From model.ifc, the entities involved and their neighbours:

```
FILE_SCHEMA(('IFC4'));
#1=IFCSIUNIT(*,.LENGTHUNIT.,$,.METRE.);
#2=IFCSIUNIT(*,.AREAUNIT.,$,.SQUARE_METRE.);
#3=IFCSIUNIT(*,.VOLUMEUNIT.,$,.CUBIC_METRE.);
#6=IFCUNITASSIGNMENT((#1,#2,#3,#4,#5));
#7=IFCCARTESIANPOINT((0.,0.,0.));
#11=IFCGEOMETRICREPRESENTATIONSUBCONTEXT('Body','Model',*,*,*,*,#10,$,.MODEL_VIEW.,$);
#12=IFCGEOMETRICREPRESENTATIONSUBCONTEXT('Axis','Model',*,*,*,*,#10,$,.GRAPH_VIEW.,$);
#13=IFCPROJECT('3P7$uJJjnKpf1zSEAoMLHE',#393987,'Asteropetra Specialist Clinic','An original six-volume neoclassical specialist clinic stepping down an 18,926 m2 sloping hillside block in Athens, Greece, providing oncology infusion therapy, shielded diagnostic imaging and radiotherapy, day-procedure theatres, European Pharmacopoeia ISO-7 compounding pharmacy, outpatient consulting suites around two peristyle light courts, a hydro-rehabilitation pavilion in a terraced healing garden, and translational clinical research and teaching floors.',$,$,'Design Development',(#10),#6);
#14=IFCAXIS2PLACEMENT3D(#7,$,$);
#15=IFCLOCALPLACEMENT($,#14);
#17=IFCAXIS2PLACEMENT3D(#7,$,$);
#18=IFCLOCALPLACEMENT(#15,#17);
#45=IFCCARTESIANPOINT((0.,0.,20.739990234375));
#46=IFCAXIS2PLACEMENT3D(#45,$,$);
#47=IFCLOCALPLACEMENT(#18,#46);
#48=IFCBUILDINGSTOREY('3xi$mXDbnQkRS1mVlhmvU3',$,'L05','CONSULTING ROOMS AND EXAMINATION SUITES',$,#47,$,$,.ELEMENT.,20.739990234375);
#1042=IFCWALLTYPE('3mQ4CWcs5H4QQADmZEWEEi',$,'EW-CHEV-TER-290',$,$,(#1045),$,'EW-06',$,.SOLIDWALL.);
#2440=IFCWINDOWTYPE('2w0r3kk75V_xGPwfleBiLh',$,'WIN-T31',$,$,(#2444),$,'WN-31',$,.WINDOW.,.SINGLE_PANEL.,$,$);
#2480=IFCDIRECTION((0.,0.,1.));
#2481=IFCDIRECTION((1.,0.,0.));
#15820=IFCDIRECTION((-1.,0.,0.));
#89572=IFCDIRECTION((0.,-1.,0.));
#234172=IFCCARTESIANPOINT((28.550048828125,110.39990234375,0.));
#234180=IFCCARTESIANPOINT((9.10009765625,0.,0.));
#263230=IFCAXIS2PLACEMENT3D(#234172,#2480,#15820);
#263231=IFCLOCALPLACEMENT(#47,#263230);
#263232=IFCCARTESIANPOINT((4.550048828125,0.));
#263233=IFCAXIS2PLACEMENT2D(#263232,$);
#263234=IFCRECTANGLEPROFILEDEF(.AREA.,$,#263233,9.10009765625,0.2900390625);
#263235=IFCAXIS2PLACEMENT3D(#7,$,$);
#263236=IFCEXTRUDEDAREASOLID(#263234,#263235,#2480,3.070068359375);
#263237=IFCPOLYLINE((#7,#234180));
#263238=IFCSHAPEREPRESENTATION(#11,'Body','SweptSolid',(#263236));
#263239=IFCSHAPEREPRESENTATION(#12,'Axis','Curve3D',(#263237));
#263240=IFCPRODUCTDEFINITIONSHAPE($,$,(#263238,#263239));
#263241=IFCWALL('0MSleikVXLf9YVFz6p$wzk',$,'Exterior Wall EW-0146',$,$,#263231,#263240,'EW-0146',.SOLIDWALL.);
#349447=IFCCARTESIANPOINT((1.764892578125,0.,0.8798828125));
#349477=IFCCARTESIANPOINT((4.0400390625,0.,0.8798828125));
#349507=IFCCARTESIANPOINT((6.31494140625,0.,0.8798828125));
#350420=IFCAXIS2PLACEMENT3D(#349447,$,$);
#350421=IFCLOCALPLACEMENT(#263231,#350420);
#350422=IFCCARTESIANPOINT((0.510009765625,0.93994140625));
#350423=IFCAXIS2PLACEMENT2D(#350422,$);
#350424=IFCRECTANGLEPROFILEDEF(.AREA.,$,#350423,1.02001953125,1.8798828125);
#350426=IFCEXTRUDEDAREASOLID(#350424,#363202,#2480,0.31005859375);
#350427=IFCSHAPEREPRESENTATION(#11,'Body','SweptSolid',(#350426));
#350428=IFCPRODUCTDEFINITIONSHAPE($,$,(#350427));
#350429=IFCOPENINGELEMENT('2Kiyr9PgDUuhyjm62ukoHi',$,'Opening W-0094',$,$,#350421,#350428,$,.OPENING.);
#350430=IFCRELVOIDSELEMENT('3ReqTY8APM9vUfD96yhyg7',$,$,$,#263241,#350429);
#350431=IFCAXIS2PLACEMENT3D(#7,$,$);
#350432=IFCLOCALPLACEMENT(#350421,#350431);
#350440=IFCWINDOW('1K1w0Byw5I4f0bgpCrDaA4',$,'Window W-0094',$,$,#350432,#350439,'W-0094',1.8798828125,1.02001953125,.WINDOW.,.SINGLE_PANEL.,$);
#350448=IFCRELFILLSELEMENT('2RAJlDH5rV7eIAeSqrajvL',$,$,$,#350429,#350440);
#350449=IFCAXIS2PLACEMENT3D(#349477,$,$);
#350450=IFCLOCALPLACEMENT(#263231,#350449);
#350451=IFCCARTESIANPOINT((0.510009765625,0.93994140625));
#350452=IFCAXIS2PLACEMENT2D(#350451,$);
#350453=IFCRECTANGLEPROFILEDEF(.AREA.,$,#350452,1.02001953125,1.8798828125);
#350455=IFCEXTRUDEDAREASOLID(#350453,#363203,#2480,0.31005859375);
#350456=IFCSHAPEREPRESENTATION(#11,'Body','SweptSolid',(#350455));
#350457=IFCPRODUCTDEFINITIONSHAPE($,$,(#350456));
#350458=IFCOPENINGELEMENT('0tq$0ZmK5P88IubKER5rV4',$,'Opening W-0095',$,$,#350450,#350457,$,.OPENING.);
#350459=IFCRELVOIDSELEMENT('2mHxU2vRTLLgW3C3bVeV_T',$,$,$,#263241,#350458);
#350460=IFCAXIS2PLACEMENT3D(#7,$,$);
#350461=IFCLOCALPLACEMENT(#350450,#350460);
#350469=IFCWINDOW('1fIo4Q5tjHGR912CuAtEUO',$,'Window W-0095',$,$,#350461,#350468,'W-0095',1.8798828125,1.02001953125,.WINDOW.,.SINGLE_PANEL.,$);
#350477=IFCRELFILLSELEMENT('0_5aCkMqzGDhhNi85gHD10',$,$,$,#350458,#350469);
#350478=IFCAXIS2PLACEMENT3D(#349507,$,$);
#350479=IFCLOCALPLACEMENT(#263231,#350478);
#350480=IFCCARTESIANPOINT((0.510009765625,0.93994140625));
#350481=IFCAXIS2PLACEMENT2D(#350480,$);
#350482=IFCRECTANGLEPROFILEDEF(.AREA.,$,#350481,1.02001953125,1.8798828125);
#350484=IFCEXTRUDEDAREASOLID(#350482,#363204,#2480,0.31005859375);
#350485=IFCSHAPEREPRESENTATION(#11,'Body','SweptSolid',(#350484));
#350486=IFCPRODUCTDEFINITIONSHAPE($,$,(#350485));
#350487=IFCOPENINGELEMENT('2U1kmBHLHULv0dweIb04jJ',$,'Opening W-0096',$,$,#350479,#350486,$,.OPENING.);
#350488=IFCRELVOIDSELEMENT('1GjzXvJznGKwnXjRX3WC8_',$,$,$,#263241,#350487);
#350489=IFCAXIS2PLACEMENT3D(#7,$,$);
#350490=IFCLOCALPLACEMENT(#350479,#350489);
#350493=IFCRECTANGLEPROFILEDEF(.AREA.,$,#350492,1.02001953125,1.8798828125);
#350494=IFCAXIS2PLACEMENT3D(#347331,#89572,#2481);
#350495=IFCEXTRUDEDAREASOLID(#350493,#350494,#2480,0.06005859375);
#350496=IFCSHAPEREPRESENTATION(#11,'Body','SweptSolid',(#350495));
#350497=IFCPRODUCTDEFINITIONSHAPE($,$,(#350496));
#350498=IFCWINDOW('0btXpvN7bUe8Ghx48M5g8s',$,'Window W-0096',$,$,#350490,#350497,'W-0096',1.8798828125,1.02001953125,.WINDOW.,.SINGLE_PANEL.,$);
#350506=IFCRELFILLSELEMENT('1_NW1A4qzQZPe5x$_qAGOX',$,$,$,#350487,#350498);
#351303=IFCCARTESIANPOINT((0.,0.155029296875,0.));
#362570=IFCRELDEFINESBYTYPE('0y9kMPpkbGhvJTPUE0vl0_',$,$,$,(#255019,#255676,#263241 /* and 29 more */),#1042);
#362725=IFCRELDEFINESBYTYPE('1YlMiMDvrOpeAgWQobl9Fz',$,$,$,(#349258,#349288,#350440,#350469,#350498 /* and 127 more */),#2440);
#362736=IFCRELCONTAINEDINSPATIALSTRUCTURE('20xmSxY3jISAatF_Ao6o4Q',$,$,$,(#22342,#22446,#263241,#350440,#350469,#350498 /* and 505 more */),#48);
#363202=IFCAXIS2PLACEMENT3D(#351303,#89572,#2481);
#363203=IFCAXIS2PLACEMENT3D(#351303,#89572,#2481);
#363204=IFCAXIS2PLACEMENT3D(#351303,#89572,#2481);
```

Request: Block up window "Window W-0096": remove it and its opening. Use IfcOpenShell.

```python
import ifcopenshell
import ifcopenshell.api.feature
import ifcopenshell.api.root
import ifcopenshell.geom
import ifcopenshell.util.shape

model = ifcopenshell.open("model.ifc")
settings = ifcopenshell.geom.settings()


def volume(element):
    """Net volume in cubic metres, openings subtracted."""
    shape = ifcopenshell.geom.create_shape(settings, element)
    return ifcopenshell.util.shape.get_volume(shape.geometry)


window = model.by_guid("0btXpvN7bUe8Ghx48M5g8s")
opening = window.FillsVoids[0].RelatingOpeningElement
wall = opening.VoidsElements[0].RelatingBuildingElement
before = volume(wall)

ifcopenshell.api.root.remove_product(model, product=window)
ifcopenshell.api.feature.remove_feature(model, feature=opening)

after = volume(wall)

print(f"wall volume {before:.3f} -> {after:.3f} m3")

model.write("model_updated.ifc")
```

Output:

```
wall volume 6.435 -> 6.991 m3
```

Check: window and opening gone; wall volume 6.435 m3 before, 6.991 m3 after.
